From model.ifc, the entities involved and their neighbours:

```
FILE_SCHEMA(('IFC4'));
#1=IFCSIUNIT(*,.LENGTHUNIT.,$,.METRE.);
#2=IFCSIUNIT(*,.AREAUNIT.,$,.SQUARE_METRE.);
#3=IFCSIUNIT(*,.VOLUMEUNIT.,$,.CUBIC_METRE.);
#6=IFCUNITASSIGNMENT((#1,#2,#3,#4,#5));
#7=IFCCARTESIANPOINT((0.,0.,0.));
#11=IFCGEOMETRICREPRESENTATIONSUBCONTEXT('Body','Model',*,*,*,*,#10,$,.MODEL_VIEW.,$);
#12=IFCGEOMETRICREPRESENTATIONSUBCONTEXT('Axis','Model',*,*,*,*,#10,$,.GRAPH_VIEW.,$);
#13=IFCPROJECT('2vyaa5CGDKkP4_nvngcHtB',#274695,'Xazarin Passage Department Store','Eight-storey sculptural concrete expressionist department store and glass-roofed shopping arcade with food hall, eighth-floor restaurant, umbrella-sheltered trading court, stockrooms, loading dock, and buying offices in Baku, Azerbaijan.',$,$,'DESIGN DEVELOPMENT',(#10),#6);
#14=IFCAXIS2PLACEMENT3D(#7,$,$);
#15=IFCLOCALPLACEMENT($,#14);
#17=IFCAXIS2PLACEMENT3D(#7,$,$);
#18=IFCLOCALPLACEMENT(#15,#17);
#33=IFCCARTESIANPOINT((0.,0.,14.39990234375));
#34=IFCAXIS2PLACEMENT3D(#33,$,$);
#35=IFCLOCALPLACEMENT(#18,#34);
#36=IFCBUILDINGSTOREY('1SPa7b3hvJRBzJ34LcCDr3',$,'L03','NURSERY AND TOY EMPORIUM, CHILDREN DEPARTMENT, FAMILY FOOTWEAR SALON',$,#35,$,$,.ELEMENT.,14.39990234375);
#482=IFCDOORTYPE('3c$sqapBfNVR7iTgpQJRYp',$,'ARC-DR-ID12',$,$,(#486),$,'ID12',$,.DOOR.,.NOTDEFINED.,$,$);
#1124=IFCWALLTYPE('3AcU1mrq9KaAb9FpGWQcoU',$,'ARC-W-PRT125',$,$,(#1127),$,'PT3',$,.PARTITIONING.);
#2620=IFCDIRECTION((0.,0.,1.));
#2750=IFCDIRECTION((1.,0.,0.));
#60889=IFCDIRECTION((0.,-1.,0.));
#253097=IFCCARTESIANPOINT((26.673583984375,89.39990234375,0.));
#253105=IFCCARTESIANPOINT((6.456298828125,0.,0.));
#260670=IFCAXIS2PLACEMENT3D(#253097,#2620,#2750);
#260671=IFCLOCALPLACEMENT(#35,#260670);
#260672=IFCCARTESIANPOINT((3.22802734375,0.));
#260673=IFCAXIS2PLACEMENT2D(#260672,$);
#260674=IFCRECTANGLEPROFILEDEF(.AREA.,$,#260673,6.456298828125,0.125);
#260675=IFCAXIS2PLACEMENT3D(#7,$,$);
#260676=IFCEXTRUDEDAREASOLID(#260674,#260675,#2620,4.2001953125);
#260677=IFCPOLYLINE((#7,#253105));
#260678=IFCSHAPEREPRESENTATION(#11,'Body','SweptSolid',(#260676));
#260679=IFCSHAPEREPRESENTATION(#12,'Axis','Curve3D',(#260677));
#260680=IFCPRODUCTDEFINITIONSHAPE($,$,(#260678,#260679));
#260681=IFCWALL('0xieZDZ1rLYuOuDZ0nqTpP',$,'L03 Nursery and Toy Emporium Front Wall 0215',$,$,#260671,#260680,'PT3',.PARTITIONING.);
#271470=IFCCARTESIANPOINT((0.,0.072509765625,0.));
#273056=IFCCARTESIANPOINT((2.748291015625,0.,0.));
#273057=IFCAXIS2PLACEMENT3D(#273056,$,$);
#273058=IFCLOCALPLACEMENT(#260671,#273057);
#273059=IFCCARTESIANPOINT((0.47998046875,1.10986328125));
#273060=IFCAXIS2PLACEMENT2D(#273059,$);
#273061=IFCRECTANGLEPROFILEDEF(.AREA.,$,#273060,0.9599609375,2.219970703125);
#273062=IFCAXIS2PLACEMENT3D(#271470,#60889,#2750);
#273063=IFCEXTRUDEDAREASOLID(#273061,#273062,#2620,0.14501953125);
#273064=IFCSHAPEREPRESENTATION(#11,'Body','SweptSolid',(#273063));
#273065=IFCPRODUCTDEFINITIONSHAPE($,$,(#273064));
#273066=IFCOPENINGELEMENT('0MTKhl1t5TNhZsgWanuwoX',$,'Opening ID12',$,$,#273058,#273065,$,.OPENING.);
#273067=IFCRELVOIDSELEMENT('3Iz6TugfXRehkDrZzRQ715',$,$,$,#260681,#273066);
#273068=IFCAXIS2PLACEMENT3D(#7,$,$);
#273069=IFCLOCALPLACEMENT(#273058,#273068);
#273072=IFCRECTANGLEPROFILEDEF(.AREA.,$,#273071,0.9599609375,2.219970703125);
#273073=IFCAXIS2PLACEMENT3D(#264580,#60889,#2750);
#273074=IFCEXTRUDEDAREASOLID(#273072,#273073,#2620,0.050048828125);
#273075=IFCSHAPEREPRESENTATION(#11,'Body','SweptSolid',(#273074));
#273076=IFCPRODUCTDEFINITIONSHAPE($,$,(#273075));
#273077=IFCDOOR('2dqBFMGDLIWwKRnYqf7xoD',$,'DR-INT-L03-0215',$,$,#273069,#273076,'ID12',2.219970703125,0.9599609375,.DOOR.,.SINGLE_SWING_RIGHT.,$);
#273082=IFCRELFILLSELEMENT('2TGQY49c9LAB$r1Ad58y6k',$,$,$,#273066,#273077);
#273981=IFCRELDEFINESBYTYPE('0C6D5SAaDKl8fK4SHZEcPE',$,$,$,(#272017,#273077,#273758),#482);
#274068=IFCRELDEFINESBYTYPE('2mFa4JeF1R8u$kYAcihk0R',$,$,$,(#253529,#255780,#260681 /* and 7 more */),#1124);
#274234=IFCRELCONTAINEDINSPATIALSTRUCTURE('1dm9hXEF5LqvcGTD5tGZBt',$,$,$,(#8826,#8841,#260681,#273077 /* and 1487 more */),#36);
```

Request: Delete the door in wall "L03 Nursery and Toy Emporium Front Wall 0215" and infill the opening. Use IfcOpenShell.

```python
import ifcopenshell
import ifcopenshell.api.feature
import ifcopenshell.api.root
import ifcopenshell.geom
import ifcopenshell.util.shape

model = ifcopenshell.open("model.ifc")
settings = ifcopenshell.geom.settings()


def volume(element):
    """Net volume in cubic metres, openings subtracted."""
    shape = ifcopenshell.geom.create_shape(settings, element)
    return ifcopenshell.util.shape.get_volume(shape.geometry)


door = model.by_guid("2dqBFMGDLIWwKRnYqf7xoD")
opening = door.FillsVoids[0].RelatingOpeningElement
wall = opening.VoidsElements[0].RelatingBuildingElement
before = volume(wall)

ifcopenshell.api.root.remove_product(model, product=door)
ifcopenshell.api.feature.remove_feature(model, feature=opening)

after = volume(wall)

print(f"wall volume {before:.3f} -> {after:.3f} m3")

model.write("model_v2.ifc")
```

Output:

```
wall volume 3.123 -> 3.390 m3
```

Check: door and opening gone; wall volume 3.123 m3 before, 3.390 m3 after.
